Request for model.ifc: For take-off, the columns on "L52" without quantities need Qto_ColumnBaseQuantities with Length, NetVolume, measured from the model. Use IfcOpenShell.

First a look at what the model holds.

```python
import ifcopenshell
import ifcopenshell.util.element
import ifcopenshell.util.unit

model = ifcopenshell.open("model.ifc")
print(model.schema)
for unit_type in ("LENGTHUNIT", "AREAUNIT", "VOLUMEUNIT"):
    print(unit_type, ifcopenshell.util.unit.calculate_unit_scale(model, unit_type))
storey = next(s for s in model.by_type("IfcBuildingStorey") if s.Name == "L52")
columns = [e for e in ifcopenshell.util.element.get_decomposition(storey) if e.is_a("IfcColumn")]
for e in sorted(columns, key=lambda e: e.id()):
    print(e.id(), e.is_a(), e.Name, list(ifcopenshell.util.element.get_psets(e, qtos_only=True)), sep=" | ")
```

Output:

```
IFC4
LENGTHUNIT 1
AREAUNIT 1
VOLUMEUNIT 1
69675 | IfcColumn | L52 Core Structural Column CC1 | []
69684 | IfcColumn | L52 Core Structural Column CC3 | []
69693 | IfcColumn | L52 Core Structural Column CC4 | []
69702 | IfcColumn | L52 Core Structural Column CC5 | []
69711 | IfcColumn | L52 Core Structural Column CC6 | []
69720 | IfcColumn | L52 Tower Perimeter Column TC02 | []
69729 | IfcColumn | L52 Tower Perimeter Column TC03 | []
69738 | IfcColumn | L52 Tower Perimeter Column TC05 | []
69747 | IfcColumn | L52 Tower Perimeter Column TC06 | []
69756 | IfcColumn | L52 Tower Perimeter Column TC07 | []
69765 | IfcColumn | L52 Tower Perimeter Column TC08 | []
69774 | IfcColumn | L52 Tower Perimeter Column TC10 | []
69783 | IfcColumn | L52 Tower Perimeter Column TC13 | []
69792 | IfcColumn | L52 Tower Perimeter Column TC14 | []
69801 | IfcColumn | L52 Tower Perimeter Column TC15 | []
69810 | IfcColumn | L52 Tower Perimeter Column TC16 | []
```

```python
import ifcopenshell
import ifcopenshell.api.pset
import ifcopenshell.geom
import ifcopenshell.util.element
import ifcopenshell.util.shape
import ifcopenshell.util.unit

model = ifcopenshell.open("model.ifc")
unit_scale = ifcopenshell.util.unit.calculate_unit_scale(model)
volume_scale = ifcopenshell.util.unit.calculate_unit_scale(model, "VOLUMEUNIT")
settings = ifcopenshell.geom.settings()

storey = next(s for s in model.by_type("IfcBuildingStorey") if s.Name == "L52")
columns = [e for e in ifcopenshell.util.element.get_decomposition(storey) if e.is_a("IfcColumn")]

for e in sorted(columns, key=lambda e: e.id()):
    if ifcopenshell.util.element.get_psets(e, qtos_only=True, should_inherit=False):
        continue
    # Geometry comes back in metres, in the element's own axes.
    shape = ifcopenshell.geom.create_shape(settings, e)
    values = {
        "Length": ifcopenshell.util.shape.get_z(shape.geometry) / unit_scale,
        "NetVolume": ifcopenshell.util.shape.get_volume(shape.geometry) / volume_scale,
    }
    qto = ifcopenshell.api.pset.add_qto(model, product=e, name="Qto_ColumnBaseQuantities")
    ifcopenshell.api.pset.edit_qto(model, qto=qto, properties=values)
    print(e.id(), {k: round(v, 3) for k, v in values.items()})

model.write("model_v2.ifc")
```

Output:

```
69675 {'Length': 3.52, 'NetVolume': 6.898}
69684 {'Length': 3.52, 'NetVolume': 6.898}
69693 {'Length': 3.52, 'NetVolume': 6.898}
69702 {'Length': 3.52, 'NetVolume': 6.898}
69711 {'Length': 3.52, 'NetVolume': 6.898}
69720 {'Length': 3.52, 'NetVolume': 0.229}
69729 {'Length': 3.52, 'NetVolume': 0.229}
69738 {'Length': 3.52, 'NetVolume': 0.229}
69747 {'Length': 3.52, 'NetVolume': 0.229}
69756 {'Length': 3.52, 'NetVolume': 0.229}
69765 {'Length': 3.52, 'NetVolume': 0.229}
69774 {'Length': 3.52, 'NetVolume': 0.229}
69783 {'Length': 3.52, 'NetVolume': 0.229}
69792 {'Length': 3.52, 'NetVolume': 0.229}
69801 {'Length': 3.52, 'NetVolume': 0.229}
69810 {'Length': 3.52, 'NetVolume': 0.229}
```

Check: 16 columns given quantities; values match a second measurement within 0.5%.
